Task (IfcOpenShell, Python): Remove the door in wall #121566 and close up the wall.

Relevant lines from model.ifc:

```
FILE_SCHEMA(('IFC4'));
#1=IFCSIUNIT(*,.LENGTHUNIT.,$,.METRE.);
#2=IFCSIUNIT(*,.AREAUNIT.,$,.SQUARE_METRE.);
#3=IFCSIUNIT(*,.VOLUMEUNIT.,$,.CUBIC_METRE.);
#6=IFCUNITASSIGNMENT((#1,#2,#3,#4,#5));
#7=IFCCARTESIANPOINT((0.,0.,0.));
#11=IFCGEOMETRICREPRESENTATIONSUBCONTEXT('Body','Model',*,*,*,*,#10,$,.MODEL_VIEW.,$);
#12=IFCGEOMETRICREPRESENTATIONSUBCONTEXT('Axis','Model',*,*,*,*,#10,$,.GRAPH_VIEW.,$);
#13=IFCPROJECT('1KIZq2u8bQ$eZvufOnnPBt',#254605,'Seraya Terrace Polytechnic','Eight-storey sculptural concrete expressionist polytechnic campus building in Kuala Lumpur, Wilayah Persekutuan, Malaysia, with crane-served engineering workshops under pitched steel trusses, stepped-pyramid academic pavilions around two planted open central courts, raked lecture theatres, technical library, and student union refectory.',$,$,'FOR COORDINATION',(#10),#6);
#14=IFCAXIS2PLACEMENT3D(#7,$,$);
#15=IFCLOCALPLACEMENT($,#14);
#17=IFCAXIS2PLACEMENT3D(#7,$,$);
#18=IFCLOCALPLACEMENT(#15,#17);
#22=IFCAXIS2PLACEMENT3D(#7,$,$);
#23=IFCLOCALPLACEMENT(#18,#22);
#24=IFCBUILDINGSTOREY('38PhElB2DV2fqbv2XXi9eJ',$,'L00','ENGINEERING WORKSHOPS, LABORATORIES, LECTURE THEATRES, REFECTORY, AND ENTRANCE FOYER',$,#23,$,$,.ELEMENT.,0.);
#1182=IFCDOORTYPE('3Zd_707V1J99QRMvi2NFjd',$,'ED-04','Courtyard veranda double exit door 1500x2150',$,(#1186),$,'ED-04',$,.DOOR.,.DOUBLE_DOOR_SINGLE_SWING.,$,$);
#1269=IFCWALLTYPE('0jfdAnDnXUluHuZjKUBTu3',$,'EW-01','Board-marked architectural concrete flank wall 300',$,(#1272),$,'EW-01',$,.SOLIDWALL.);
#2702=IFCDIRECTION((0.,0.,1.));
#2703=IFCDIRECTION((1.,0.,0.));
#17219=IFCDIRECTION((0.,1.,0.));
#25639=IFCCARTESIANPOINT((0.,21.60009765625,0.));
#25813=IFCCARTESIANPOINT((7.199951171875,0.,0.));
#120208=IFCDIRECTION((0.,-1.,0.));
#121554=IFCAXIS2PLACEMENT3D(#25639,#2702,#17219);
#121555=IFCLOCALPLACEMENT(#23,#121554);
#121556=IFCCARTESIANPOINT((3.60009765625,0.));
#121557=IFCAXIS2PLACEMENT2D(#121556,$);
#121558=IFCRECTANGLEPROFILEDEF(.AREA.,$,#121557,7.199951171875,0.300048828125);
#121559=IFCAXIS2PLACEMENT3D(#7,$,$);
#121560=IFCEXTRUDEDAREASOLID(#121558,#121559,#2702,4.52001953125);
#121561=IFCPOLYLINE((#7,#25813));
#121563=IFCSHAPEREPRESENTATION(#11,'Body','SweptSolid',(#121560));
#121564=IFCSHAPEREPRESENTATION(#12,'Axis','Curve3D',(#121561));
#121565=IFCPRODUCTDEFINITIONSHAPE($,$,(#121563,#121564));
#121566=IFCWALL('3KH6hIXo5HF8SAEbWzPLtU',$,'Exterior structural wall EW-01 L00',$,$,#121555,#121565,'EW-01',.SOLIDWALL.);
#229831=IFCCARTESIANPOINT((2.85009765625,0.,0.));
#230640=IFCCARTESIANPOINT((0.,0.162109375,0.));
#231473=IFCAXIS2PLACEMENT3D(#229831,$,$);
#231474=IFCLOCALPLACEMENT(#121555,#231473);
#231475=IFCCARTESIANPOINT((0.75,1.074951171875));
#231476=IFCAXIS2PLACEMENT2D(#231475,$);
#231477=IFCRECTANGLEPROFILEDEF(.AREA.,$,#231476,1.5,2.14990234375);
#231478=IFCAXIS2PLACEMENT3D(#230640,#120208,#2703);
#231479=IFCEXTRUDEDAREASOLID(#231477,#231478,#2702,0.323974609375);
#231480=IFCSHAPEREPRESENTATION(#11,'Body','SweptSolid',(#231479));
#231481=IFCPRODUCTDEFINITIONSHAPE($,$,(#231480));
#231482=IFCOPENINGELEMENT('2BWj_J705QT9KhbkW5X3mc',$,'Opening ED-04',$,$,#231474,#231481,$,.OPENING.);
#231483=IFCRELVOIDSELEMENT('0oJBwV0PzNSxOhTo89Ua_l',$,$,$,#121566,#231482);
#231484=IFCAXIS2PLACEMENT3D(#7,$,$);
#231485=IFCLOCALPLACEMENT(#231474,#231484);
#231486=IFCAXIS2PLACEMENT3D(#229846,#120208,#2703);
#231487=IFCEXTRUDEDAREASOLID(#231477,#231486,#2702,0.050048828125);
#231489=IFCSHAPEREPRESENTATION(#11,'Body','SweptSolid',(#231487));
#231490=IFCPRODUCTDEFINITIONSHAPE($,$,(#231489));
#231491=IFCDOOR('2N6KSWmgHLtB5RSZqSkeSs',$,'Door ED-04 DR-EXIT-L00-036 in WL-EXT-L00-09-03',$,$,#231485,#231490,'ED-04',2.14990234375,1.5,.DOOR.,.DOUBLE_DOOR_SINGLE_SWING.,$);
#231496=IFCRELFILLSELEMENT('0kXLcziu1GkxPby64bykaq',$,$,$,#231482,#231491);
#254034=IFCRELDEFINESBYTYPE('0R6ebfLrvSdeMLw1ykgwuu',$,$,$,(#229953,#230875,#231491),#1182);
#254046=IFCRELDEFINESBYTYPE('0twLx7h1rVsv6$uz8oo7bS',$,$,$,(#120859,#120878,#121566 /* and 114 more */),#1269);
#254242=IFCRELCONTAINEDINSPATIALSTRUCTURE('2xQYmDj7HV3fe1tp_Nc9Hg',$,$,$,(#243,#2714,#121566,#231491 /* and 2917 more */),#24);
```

```python
import ifcopenshell
import ifcopenshell.api.feature
import ifcopenshell.api.root
import ifcopenshell.geom
import ifcopenshell.util.shape

model = ifcopenshell.open("model.ifc")
settings = ifcopenshell.geom.settings()


def volume(element):
    """Net volume in cubic metres, openings subtracted."""
    shape = ifcopenshell.geom.create_shape(settings, element)
    return ifcopenshell.util.shape.get_volume(shape.geometry)


door = model.by_guid("2N6KSWmgHLtB5RSZqSkeSs")
opening = door.FillsVoids[0].RelatingOpeningElement
wall = opening.VoidsElements[0].RelatingBuildingElement
before = volume(wall)

ifcopenshell.api.root.remove_product(model, product=door)
ifcopenshell.api.feature.remove_feature(model, feature=opening)

after = volume(wall)

print(f"wall volume {before:.3f} -> {after:.3f} m3")

model.write("model_updated.ifc")
```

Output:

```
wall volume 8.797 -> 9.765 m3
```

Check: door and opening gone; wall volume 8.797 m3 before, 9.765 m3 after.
